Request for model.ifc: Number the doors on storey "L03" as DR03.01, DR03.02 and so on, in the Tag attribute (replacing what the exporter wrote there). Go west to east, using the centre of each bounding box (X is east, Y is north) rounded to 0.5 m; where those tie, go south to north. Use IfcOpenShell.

First a look at what the model holds.

```python
import ifcopenshell
import ifcopenshell.util.element
import ifcopenshell.util.placement

model = ifcopenshell.open("model.ifc")
print(model.schema)
storey = next(s for s in model.by_type("IfcBuildingStorey") if s.Name == "L03")
doors = [e for e in ifcopenshell.util.element.get_decomposition(storey) if e.is_a("IfcDoor")]
for e in sorted(doors, key=lambda e: e.id()):
    origin = ifcopenshell.util.placement.get_local_placement(e.ObjectPlacement)[:3, 3]
    print(e.id(), e.Tag, e.Name, origin.round(2) + 0.0, sep=" | ")
```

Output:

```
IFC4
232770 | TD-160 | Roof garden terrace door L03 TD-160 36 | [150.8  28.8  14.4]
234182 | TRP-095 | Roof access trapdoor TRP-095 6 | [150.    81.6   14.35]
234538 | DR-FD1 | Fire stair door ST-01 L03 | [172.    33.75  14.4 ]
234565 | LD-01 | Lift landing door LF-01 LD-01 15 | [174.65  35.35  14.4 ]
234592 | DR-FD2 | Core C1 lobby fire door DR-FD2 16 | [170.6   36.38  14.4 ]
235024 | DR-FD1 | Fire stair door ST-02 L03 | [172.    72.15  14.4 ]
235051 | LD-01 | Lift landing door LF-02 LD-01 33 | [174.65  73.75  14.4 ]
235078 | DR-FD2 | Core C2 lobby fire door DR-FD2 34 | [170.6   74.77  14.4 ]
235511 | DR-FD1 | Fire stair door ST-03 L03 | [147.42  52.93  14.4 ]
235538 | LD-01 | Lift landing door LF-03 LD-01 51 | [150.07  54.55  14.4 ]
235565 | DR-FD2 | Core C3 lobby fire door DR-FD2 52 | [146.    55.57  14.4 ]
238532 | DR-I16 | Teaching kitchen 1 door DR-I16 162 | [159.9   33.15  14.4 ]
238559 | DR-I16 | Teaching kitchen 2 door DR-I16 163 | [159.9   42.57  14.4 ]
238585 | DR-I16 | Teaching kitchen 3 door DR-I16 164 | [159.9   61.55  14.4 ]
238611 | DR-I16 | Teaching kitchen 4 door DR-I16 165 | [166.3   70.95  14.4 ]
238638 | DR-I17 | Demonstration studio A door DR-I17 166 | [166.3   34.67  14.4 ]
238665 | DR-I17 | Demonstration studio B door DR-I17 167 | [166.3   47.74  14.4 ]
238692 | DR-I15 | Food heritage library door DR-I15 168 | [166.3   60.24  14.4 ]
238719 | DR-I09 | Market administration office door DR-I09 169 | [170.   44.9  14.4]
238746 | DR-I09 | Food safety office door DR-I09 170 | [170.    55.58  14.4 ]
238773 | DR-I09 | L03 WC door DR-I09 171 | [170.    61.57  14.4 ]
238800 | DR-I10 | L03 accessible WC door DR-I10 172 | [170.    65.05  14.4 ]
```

```python
import ifcopenshell
import ifcopenshell.geom
import ifcopenshell.util.element
import ifcopenshell.util.shape

model = ifcopenshell.open("model.ifc")
settings = ifcopenshell.geom.settings()
settings.set("use-world-coords", True)


def centre(element):
    shape = ifcopenshell.geom.create_shape(settings, element)
    return ifcopenshell.util.shape.get_bbox_centroid(shape.geometry)


storey = next(s for s in model.by_type("IfcBuildingStorey") if s.Name == "L03")
doors = [e for e in ifcopenshell.util.element.get_decomposition(storey) if e.is_a("IfcDoor")]

# Insertion points can sit at a corner or the storey origin, so sort by the geometry (in metres).
centres = {e: centre(e) for e in doors}
doors.sort(key=lambda e: (round(centres[e][0] / 0.5), centres[e][1]))

for i, e in enumerate(doors, start=1):
    number = f"DR03.{i:02d}"
    e.Tag = number
    print(e.id(), number)

model.write("model_rev.ifc")
```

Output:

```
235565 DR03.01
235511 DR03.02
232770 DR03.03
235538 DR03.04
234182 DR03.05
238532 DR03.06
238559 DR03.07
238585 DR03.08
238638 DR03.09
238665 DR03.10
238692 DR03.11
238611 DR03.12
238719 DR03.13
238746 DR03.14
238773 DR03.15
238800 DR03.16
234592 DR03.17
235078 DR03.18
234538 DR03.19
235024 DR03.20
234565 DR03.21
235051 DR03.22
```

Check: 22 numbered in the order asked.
